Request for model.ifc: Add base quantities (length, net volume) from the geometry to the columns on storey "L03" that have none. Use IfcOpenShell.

First a look at what the model holds.

```python
import ifcopenshell
import ifcopenshell.util.element
import ifcopenshell.util.unit

model = ifcopenshell.open("model.ifc")
print(model.schema)
for unit_type in ("LENGTHUNIT", "AREAUNIT", "VOLUMEUNIT"):
    print(unit_type, ifcopenshell.util.unit.calculate_unit_scale(model, unit_type))
storey = next(s for s in model.by_type("IfcBuildingStorey") if s.Name == "L03")
columns = [e for e in ifcopenshell.util.element.get_decomposition(storey) if e.is_a("IfcColumn")]
for e in sorted(columns, key=lambda e: e.id()):
    print(e.id(), e.is_a(), e.Name, list(ifcopenshell.util.element.get_psets(e, qtos_only=True)), sep=" | ")
```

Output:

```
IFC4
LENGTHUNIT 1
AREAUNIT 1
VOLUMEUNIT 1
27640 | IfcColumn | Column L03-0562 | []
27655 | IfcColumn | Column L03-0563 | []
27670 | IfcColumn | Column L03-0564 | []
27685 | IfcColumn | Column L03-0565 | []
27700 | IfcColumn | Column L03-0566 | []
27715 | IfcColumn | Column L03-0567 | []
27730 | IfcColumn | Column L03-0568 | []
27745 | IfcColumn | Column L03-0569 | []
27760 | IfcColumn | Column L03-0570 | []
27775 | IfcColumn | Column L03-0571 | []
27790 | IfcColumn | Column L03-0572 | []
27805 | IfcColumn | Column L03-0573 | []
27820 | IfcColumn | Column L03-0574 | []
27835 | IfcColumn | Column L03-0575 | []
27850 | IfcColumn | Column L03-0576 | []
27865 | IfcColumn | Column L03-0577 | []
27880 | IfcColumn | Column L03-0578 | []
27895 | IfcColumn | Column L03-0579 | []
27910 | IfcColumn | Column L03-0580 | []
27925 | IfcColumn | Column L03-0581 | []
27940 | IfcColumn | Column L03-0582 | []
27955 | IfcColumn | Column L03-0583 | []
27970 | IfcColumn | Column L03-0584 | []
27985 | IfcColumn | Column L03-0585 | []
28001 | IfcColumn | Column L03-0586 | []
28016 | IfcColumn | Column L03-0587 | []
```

```python
import ifcopenshell
import ifcopenshell.api.pset
import ifcopenshell.geom
import ifcopenshell.util.element
import ifcopenshell.util.shape
import ifcopenshell.util.unit

model = ifcopenshell.open("model.ifc")
unit_scale = ifcopenshell.util.unit.calculate_unit_scale(model)
volume_scale = ifcopenshell.util.unit.calculate_unit_scale(model, "VOLUMEUNIT")
settings = ifcopenshell.geom.settings()

storey = next(s for s in model.by_type("IfcBuildingStorey") if s.Name == "L03")
columns = [e for e in ifcopenshell.util.element.get_decomposition(storey) if e.is_a("IfcColumn")]

for e in sorted(columns, key=lambda e: e.id()):
    if ifcopenshell.util.element.get_psets(e, qtos_only=True, should_inherit=False):
        continue
    # Geometry comes back in metres, in the element's own axes.
    shape = ifcopenshell.geom.create_shape(settings, e)
    values = {
        "Length": ifcopenshell.util.shape.get_z(shape.geometry) / unit_scale,
        "NetVolume": ifcopenshell.util.shape.get_volume(shape.geometry) / volume_scale,
    }
    qto = ifcopenshell.api.pset.add_qto(model, product=e, name="Qto_ColumnBaseQuantities")
    ifcopenshell.api.pset.edit_qto(model, qto=qto, properties=values)
    print(e.id(), {k: round(v, 3) for k, v in values.items()})

model.write("model_rev.ifc")
```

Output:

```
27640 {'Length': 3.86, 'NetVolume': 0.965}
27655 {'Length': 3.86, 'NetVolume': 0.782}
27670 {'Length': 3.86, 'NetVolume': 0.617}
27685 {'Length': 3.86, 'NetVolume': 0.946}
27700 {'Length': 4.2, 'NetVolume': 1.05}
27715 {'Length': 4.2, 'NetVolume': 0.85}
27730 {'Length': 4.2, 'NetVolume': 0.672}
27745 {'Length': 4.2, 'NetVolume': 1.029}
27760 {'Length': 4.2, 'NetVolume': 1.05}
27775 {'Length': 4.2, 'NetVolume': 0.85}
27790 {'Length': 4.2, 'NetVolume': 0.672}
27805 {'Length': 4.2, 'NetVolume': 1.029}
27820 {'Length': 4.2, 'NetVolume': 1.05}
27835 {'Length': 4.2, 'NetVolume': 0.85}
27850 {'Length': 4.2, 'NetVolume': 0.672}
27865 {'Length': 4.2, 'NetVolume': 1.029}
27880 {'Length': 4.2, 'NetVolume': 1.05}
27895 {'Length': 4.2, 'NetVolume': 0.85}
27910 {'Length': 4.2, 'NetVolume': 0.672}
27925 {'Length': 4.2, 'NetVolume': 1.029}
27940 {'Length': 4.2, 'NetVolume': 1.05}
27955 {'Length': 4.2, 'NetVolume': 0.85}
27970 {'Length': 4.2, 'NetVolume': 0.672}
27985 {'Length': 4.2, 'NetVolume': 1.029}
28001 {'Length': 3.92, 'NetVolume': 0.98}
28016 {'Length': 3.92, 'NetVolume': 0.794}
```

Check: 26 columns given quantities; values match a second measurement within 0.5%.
